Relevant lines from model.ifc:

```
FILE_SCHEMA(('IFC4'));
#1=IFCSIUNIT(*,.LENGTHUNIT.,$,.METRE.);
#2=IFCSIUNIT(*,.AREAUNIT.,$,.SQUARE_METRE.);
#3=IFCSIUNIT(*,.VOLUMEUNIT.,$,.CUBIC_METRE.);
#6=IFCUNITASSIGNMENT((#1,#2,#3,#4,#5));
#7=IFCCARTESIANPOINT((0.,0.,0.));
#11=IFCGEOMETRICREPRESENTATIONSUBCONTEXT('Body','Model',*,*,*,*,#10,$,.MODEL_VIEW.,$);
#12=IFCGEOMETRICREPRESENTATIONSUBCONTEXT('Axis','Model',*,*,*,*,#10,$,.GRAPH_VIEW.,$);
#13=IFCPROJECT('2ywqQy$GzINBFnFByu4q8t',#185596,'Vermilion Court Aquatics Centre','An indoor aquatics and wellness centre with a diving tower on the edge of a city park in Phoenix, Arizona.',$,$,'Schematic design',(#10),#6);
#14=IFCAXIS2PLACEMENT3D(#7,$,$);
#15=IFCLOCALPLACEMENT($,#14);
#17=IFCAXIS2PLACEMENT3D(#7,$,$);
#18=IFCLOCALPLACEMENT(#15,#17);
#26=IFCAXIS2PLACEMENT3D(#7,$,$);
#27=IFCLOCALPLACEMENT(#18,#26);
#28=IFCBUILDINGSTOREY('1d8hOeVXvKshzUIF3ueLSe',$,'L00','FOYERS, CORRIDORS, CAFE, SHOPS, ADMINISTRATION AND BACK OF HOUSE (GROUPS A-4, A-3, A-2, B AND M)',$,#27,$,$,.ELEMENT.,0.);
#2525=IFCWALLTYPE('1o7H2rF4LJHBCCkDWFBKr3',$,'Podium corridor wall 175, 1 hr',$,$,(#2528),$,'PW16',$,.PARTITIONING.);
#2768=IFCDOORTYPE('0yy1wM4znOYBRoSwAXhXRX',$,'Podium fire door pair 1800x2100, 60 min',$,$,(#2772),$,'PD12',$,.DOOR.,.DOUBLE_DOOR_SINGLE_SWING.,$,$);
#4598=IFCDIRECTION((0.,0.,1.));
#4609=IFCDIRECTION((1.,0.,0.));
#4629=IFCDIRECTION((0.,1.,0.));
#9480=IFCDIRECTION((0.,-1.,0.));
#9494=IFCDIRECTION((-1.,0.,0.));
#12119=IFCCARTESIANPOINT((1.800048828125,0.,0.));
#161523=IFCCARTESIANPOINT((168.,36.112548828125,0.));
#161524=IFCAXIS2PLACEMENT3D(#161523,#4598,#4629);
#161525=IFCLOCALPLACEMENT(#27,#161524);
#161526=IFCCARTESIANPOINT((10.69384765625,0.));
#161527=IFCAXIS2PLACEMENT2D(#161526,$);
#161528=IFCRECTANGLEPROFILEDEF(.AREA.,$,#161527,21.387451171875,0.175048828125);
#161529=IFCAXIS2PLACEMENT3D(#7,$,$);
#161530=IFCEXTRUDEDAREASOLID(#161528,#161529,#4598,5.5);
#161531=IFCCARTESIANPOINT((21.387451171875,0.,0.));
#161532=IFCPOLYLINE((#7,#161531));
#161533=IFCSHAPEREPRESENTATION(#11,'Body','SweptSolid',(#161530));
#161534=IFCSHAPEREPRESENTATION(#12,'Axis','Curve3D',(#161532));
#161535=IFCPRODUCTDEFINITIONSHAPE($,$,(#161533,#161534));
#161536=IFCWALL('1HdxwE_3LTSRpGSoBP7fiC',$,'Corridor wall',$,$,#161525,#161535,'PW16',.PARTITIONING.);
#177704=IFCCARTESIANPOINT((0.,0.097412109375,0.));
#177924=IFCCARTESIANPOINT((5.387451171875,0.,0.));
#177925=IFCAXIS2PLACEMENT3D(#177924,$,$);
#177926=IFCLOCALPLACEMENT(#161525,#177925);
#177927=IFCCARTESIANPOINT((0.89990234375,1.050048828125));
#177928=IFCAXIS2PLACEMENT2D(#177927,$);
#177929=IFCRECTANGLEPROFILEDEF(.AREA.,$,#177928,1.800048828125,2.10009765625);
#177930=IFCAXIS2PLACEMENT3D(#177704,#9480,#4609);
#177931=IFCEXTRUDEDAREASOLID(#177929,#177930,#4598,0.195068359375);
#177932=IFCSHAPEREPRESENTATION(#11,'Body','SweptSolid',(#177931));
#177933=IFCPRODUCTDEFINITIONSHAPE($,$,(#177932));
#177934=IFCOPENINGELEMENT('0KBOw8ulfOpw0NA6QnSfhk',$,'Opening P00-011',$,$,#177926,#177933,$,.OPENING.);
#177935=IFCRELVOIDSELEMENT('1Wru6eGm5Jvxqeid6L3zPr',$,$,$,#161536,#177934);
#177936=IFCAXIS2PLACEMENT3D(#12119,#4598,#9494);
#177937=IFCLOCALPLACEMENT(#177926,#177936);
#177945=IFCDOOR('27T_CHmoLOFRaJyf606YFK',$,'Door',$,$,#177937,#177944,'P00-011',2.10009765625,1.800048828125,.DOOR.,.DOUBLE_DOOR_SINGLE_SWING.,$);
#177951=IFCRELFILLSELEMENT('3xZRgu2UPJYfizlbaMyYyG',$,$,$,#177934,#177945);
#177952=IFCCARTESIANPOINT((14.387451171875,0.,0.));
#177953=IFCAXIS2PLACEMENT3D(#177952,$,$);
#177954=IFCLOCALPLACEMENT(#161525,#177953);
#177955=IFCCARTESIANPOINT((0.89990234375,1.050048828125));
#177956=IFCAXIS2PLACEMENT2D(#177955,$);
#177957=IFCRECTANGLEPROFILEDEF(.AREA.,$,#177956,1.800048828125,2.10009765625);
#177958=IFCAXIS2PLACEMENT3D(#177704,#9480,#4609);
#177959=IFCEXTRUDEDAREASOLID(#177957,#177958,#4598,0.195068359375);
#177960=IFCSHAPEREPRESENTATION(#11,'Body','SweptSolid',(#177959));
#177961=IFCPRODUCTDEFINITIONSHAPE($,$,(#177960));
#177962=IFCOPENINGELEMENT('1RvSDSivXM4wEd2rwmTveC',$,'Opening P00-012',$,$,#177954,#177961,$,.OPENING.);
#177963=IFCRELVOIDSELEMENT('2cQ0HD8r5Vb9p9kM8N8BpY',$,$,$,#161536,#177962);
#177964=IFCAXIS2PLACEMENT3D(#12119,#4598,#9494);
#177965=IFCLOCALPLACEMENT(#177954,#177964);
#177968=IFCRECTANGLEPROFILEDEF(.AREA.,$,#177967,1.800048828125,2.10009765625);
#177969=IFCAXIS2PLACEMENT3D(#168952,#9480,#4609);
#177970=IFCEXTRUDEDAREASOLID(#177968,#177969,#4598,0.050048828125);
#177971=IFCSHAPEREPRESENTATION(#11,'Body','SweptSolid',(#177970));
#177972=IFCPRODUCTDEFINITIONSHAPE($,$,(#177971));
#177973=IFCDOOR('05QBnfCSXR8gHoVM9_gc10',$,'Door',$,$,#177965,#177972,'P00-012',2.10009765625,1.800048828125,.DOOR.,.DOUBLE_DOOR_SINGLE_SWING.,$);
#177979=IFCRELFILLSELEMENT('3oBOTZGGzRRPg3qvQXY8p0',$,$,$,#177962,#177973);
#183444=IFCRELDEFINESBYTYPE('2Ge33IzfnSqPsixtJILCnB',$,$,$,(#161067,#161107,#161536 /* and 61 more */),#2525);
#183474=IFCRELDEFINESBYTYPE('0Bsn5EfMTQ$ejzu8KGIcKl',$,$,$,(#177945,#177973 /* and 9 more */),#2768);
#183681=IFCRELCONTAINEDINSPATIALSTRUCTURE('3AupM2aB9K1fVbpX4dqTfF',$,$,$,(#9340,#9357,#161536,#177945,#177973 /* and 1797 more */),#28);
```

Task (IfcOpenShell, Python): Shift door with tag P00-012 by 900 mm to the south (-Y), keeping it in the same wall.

```python
import ifcopenshell
import ifcopenshell.api.geometry
import ifcopenshell.util.placement

model = ifcopenshell.open("model.ifc")

door = model.by_guid("05QBnfCSXR8gHoVM9_gc10")
opening = door.FillsVoids[0].RelatingOpeningElement
wall = opening.VoidsElements[0].RelatingBuildingElement

wall_matrix = ifcopenshell.util.placement.get_local_placement(wall.ObjectPlacement)
shift = wall_matrix[:3, 0] * -0.9
before = ifcopenshell.util.placement.get_local_placement(door.ObjectPlacement)[:3, 3].copy()

# The door is placed relative to its opening, so it follows when the opening moves.
matrix = ifcopenshell.util.placement.get_local_placement(opening.ObjectPlacement)
matrix[:3, 3] += shift
ifcopenshell.api.geometry.edit_object_placement(
    model, product=opening, matrix=matrix, is_si=False, should_transform_children=True
)

after = ifcopenshell.util.placement.get_local_placement(door.ObjectPlacement)[:3, 3]
print("door moved by", (after - before).round(3) + 0.0)

model.write("model-out.ifc")
```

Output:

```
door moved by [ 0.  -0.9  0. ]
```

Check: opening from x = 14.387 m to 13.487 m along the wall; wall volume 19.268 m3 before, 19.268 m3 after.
